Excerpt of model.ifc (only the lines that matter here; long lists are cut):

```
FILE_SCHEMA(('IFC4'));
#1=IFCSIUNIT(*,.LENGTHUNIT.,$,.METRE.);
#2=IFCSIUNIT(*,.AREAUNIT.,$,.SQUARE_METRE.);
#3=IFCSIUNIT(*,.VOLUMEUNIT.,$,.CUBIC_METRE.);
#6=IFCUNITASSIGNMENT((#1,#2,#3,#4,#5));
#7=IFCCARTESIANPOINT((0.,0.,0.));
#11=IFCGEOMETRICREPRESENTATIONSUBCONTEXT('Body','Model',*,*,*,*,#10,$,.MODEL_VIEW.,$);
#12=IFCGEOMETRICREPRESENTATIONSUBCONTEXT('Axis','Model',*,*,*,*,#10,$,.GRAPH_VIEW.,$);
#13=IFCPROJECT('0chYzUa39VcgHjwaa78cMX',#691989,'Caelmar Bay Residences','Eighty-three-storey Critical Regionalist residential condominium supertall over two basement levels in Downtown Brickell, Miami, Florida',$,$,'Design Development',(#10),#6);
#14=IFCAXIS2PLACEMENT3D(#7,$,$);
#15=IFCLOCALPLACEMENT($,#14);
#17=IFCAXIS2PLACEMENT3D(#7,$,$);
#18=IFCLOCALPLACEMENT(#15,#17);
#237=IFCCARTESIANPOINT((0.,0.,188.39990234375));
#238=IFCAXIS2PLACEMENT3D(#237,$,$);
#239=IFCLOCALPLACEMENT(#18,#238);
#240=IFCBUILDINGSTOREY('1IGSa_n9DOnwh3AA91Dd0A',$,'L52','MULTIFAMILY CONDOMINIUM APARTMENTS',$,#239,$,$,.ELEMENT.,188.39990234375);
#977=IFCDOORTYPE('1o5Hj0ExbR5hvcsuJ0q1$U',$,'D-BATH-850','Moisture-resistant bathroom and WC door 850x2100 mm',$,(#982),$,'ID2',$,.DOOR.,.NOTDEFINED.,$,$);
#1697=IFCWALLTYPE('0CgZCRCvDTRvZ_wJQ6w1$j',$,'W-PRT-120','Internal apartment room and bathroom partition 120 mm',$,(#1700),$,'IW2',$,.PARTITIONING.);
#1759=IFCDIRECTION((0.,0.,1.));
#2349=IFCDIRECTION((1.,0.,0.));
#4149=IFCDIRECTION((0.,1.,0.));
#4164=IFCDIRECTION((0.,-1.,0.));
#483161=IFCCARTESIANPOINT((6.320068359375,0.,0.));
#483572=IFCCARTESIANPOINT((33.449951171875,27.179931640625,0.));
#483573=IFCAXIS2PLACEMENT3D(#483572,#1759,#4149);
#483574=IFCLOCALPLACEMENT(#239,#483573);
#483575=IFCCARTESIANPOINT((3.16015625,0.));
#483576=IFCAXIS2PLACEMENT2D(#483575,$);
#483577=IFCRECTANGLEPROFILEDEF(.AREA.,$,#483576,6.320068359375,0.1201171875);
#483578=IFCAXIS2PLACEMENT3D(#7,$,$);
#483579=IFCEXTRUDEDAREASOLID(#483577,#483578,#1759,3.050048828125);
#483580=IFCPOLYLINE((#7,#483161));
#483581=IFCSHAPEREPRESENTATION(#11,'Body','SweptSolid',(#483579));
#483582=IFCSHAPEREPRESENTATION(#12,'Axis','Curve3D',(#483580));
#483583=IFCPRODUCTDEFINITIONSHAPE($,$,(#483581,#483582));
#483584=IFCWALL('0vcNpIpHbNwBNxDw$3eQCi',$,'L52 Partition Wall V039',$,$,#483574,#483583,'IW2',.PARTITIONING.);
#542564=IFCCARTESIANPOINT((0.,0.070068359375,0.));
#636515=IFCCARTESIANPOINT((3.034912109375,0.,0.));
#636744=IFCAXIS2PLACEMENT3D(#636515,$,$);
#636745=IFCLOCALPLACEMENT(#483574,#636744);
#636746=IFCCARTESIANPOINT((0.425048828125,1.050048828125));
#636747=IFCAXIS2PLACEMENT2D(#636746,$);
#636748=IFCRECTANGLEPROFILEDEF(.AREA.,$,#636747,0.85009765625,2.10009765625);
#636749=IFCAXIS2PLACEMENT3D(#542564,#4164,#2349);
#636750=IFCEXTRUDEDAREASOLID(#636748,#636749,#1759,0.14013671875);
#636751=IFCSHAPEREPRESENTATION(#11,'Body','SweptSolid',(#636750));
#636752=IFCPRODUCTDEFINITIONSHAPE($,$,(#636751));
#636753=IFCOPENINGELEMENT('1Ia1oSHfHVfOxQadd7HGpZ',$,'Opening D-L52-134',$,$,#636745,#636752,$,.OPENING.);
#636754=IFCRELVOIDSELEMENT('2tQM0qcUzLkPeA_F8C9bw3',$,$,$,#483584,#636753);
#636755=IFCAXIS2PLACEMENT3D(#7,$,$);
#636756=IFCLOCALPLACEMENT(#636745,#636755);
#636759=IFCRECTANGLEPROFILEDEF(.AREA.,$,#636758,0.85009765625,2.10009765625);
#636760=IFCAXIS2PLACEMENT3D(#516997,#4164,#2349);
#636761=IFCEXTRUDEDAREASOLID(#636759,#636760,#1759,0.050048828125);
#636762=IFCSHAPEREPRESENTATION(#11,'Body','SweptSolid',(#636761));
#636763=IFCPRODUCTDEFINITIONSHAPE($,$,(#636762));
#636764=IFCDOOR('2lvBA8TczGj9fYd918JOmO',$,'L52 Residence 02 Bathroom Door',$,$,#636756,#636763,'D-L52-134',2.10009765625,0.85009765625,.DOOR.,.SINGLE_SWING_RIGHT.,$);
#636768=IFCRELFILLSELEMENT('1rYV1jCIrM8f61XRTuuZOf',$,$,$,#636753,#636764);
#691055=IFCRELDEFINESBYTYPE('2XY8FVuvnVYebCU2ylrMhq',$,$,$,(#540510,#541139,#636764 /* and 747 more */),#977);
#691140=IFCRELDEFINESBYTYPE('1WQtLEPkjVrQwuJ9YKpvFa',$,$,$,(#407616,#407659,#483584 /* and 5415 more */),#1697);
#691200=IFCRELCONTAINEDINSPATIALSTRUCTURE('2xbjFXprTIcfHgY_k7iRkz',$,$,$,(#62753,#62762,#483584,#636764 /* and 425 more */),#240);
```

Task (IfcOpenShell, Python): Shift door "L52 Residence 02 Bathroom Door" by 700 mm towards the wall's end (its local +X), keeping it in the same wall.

```python
import ifcopenshell
import ifcopenshell.api.geometry
import ifcopenshell.util.placement

model = ifcopenshell.open("model.ifc")

door = model.by_guid("2lvBA8TczGj9fYd918JOmO")
opening = door.FillsVoids[0].RelatingOpeningElement
wall = opening.VoidsElements[0].RelatingBuildingElement

wall_matrix = ifcopenshell.util.placement.get_local_placement(wall.ObjectPlacement)
shift = wall_matrix[:3, 0] * 0.7
before = ifcopenshell.util.placement.get_local_placement(door.ObjectPlacement)[:3, 3].copy()

# The door is placed relative to its opening, so it follows when the opening moves.
matrix = ifcopenshell.util.placement.get_local_placement(opening.ObjectPlacement)
matrix[:3, 3] += shift
ifcopenshell.api.geometry.edit_object_placement(
    model, product=opening, matrix=matrix, is_si=False, should_transform_children=True
)

after = ifcopenshell.util.placement.get_local_placement(door.ObjectPlacement)[:3, 3]
print("door moved by", (after - before).round(3) + 0.0)

model.write("model_updated.ifc")
```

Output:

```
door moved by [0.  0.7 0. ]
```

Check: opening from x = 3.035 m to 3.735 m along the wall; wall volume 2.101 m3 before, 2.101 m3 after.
